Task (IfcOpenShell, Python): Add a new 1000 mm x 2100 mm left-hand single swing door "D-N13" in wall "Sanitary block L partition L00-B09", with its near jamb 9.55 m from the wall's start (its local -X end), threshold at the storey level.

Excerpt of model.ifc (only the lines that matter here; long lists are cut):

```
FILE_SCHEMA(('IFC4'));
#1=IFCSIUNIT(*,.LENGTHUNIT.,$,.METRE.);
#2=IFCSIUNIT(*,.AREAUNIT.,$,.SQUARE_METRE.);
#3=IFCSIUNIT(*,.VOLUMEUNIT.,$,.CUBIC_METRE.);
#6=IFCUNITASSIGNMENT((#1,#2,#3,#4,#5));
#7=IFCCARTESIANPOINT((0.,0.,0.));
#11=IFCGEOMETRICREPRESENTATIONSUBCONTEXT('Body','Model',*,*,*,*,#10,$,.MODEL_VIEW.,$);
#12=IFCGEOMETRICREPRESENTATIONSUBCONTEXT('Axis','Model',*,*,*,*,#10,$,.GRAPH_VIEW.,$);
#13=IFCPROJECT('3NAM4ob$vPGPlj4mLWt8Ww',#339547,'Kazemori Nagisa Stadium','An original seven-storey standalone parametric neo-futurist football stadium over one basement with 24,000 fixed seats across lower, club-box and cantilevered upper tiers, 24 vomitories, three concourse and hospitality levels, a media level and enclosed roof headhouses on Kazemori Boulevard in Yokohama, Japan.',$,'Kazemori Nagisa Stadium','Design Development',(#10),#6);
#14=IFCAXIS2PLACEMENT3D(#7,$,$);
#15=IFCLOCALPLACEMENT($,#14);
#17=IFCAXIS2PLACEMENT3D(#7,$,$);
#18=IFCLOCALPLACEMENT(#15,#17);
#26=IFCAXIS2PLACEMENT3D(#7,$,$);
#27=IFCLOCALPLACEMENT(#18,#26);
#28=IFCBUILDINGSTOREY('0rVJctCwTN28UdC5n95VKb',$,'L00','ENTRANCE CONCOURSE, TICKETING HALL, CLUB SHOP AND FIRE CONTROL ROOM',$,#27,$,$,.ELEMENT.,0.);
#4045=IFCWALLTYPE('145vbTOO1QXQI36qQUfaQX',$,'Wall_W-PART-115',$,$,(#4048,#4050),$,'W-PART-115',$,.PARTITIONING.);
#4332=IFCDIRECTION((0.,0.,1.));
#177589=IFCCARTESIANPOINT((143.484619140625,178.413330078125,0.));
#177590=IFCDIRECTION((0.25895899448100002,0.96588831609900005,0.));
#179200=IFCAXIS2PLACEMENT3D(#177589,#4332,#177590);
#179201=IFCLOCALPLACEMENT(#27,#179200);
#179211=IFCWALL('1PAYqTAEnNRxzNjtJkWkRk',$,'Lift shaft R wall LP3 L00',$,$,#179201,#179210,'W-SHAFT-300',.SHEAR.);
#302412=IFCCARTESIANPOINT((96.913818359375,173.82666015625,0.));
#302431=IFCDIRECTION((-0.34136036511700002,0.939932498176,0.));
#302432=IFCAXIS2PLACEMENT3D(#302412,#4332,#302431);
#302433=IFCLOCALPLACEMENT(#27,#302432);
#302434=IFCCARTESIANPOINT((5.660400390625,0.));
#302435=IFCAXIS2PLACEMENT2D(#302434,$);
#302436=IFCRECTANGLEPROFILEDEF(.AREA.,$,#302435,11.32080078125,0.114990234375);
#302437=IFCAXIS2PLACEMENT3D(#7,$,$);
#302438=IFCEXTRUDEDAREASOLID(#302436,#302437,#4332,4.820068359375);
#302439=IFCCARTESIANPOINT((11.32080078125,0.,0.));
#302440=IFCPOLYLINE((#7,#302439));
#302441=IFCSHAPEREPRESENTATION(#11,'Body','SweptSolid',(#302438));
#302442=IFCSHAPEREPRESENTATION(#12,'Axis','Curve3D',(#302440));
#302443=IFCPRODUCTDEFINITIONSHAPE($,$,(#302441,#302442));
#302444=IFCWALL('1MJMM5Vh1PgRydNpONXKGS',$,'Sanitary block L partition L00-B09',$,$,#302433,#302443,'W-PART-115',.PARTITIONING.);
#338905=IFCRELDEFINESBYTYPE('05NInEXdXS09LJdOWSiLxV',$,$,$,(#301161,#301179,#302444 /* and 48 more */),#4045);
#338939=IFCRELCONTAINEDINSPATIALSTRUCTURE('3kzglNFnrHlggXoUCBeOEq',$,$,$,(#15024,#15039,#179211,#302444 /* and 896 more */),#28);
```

```python
import numpy as np
import ifcopenshell
import ifcopenshell.api.feature
import ifcopenshell.api.geometry
import ifcopenshell.api.root
import ifcopenshell.api.spatial
import ifcopenshell.geom
import ifcopenshell.util.element
import ifcopenshell.util.placement
import ifcopenshell.util.representation
import ifcopenshell.util.shape
import ifcopenshell.util.unit

model = ifcopenshell.open("model.ifc")
unit_scale = ifcopenshell.util.unit.calculate_unit_scale(model)
settings = ifcopenshell.geom.settings()


def volume(element):
    """Net volume in cubic metres, openings subtracted."""
    shape = ifcopenshell.geom.create_shape(settings, element)
    return ifcopenshell.util.shape.get_volume(shape.geometry)


wall = model.by_id(302444)
storey = ifcopenshell.util.element.get_container(wall, ifc_class="IfcBuildingStorey")
context = ifcopenshell.util.representation.get_context(model, "Model", "Body", "MODEL_VIEW")
before = volume(wall)

width, height, from_end, sill = 1, 2.1, 9.55, 0.0  # metres

# The wall runs along its own X axis, and the end named is its -X end.
wall_shape = ifcopenshell.geom.create_shape(settings, wall)
x, y, z = ifcopenshell.util.shape.get_vertices(wall_shape.geometry).T
start = x.min() + from_end
face, thickness = float(y.min()), float(y.max() - y.min())
wall_matrix = ifcopenshell.util.placement.get_local_placement(wall.ObjectPlacement)
level = ifcopenshell.util.placement.get_local_placement(storey.ObjectPlacement)[2, 3]


def in_wall(x, y):
    """Placement at x, y metres in the wall's axes, at sill height."""
    matrix = wall_matrix.copy()
    matrix[:, 3] = wall_matrix @ np.array([x / unit_scale, y / unit_scale, 0.0, 1.0])
    matrix[2, 3] = level + sill / unit_scale
    return matrix


# Opening: a box that overshoots both wall faces by 50 mm.
opening = ifcopenshell.api.root.create_entity(model, ifc_class="IfcOpeningElement", predefined_type="OPENING")
box = ifcopenshell.api.geometry.add_wall_representation(
    model, context=context, length=width, height=height, thickness=thickness + 0.1
)
ifcopenshell.api.geometry.assign_representation(model, product=opening, representation=box)
ifcopenshell.api.geometry.edit_object_placement(model, product=opening, matrix=in_wall(start, face - 0.05), is_si=False)
ifcopenshell.api.feature.add_feature(model, feature=opening, element=wall)

door = ifcopenshell.api.root.create_entity(model, ifc_class="IfcDoor", name="D-N13", predefined_type="DOOR")
door.OverallWidth, door.OverallHeight = width / unit_scale, height / unit_scale
door.OperationType = "SINGLE_SWING_LEFT"
body = ifcopenshell.api.geometry.add_door_representation(
    model,
    context=context,
    overall_width=door.OverallWidth,
    overall_height=door.OverallHeight,
    operation_type="SINGLE_SWING_LEFT",
    lining_properties={"LiningDepth": thickness / unit_scale, "ThresholdDepth": thickness / unit_scale},
)
ifcopenshell.api.geometry.assign_representation(model, product=door, representation=body)
ifcopenshell.api.spatial.assign_container(model, products=[door], relating_structure=storey)
ifcopenshell.api.feature.add_filling(model, opening=opening, element=door)

# The lining spans the wall, so the door starts at the wall face.
ifcopenshell.api.geometry.edit_object_placement(model, product=door, matrix=in_wall(start, face), is_si=False)

after = volume(wall)

print(f"wall volume {before:.3f} -> {after:.3f} m3")

model.write("model_v2.ifc")
```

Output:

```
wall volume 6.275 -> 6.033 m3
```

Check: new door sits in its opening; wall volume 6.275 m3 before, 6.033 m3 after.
